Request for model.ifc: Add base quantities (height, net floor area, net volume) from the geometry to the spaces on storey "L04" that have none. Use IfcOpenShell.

First a look at what the model holds.

```python
import ifcopenshell
import ifcopenshell.util.element
import ifcopenshell.util.unit

model = ifcopenshell.open("model.ifc")
print(model.schema)
for unit_type in ("LENGTHUNIT", "AREAUNIT", "VOLUMEUNIT"):
    print(unit_type, ifcopenshell.util.unit.calculate_unit_scale(model, unit_type))
storey = next(s for s in model.by_type("IfcBuildingStorey") if s.Name == "L04")
spaces = [e for e in ifcopenshell.util.element.get_decomposition(storey) if e.is_a("IfcSpace")]
for e in sorted(spaces, key=lambda e: e.id()):
    print(e.id(), e.is_a(), e.Name, list(ifcopenshell.util.element.get_psets(e, qtos_only=True)), sep=" | ")
```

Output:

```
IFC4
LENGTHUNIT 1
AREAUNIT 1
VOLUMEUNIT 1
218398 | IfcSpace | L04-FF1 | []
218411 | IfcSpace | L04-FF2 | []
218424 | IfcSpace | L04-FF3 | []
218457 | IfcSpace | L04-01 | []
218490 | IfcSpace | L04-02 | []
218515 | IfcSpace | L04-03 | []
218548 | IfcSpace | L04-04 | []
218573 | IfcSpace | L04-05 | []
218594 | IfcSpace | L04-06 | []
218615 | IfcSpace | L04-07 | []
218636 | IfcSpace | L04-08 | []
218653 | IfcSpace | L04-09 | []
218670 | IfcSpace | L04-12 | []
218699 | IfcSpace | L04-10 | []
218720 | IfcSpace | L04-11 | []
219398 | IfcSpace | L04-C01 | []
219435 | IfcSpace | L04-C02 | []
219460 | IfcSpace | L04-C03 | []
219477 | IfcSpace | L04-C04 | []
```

```python
import ifcopenshell
import ifcopenshell.api.pset
import ifcopenshell.geom
import ifcopenshell.util.element
import ifcopenshell.util.shape
import ifcopenshell.util.unit

model = ifcopenshell.open("model.ifc")
unit_scale = ifcopenshell.util.unit.calculate_unit_scale(model)
area_scale = ifcopenshell.util.unit.calculate_unit_scale(model, "AREAUNIT")
volume_scale = ifcopenshell.util.unit.calculate_unit_scale(model, "VOLUMEUNIT")
settings = ifcopenshell.geom.settings()

storey = next(s for s in model.by_type("IfcBuildingStorey") if s.Name == "L04")
spaces = [e for e in ifcopenshell.util.element.get_decomposition(storey) if e.is_a("IfcSpace")]

for e in sorted(spaces, key=lambda e: e.id()):
    if ifcopenshell.util.element.get_psets(e, qtos_only=True, should_inherit=False):
        continue
    # Geometry comes back in metres, in the element's own axes.
    shape = ifcopenshell.geom.create_shape(settings, e)
    values = {
        "Height": ifcopenshell.util.shape.get_z(shape.geometry) / unit_scale,
        "NetFloorArea": ifcopenshell.util.shape.get_footprint_area(shape.geometry) / area_scale,
        "NetVolume": ifcopenshell.util.shape.get_volume(shape.geometry) / volume_scale,
    }
    qto = ifcopenshell.api.pset.add_qto(model, product=e, name="Qto_SpaceBaseQuantities")
    ifcopenshell.api.pset.edit_qto(model, qto=qto, properties=values)
    print(e.id(), {k: round(v, 3) for k, v in values.items()})

model.write("model_rev.ifc")
```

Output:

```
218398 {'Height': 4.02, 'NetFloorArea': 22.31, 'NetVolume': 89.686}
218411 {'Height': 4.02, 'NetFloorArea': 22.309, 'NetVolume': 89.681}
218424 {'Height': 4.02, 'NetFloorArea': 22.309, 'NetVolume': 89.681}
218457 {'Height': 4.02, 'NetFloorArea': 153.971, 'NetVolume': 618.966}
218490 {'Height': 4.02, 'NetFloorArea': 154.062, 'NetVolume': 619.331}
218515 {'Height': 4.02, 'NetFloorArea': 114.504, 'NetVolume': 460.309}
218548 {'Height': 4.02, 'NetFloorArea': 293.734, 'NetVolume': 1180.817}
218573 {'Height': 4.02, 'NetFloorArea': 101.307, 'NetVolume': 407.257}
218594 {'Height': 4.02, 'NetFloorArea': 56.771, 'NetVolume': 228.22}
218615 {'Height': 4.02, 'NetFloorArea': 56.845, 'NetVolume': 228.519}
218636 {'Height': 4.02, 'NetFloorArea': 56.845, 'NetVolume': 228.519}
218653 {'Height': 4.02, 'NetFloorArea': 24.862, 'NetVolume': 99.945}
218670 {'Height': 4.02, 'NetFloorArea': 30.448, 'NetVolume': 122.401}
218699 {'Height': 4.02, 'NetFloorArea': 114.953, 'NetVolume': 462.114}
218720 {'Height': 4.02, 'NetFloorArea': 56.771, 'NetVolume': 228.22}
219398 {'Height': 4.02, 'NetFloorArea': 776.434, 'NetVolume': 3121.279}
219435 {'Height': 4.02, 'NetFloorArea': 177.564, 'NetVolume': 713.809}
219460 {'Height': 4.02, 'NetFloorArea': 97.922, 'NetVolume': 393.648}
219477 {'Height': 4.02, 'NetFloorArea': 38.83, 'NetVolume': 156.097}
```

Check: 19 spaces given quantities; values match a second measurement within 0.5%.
